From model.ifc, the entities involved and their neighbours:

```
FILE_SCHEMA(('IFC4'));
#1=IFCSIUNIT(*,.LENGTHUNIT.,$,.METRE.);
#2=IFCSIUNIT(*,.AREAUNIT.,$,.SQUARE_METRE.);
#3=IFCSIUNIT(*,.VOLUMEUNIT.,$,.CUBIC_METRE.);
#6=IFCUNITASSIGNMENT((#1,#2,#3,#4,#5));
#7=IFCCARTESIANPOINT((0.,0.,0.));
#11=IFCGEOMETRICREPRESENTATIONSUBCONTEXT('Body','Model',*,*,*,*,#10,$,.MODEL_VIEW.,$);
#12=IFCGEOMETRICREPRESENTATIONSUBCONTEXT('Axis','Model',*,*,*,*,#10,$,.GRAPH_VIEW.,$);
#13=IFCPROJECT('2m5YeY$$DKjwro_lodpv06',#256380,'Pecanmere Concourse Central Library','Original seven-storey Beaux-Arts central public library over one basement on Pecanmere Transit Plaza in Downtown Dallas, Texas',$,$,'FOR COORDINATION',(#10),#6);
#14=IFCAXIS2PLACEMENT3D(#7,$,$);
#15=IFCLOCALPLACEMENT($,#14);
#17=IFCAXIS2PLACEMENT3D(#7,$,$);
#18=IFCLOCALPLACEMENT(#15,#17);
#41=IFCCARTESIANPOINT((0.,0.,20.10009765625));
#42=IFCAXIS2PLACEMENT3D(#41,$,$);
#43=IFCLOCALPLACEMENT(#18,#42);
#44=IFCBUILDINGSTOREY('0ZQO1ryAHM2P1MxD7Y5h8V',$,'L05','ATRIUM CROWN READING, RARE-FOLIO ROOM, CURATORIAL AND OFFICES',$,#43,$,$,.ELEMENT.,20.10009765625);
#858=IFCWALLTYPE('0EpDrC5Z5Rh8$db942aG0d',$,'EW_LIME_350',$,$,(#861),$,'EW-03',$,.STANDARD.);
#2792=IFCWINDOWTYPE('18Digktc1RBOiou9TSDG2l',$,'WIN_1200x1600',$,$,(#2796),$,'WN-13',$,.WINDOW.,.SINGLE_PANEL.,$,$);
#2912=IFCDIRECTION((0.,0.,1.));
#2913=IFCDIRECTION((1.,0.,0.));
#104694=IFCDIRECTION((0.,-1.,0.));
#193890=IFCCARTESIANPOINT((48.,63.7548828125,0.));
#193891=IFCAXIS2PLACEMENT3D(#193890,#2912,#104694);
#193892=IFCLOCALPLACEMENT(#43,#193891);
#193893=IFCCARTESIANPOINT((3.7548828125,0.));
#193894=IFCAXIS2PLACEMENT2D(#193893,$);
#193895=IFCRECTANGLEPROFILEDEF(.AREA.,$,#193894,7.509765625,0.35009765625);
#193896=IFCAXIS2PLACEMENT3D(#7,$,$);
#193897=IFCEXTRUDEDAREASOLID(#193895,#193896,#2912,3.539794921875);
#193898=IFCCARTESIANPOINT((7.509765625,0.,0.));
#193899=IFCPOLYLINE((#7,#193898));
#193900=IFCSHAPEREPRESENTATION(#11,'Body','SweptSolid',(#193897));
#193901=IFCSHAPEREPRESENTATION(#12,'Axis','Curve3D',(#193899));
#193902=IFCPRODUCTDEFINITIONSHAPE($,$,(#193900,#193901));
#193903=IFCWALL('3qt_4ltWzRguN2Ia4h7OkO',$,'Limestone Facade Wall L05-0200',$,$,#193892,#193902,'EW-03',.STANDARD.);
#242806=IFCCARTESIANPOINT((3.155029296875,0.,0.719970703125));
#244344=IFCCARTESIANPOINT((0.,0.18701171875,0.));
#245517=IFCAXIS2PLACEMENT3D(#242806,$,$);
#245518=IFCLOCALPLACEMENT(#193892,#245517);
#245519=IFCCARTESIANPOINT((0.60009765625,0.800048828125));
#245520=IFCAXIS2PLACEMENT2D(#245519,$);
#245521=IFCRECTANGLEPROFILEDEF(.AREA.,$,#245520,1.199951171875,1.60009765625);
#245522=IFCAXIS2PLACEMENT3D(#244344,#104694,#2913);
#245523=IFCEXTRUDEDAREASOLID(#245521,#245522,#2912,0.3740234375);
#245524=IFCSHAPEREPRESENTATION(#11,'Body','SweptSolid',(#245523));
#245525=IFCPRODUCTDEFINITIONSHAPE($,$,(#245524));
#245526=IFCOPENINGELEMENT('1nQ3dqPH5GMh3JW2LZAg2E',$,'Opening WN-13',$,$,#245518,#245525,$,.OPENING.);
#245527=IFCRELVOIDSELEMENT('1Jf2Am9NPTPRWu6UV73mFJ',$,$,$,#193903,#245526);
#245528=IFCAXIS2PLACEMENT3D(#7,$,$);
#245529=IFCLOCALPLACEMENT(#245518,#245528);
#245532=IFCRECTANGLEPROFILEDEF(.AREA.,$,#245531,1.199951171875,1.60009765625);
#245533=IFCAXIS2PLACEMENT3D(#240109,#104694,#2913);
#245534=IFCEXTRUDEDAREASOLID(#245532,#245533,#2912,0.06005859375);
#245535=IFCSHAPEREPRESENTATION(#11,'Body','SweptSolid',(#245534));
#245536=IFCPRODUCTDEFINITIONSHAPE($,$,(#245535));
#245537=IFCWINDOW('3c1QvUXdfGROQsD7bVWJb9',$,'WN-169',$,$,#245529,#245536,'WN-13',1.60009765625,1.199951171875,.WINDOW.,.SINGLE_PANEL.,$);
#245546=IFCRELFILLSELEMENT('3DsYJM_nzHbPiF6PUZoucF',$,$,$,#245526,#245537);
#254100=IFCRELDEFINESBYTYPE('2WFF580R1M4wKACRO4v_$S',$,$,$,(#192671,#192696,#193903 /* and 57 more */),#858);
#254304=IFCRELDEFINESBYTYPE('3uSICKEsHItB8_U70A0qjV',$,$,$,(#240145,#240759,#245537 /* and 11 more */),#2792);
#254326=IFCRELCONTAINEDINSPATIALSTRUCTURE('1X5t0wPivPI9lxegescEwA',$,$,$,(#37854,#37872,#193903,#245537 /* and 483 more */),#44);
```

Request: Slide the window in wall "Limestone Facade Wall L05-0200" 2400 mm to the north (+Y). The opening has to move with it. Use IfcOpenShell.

```python
import ifcopenshell
import ifcopenshell.api.geometry
import ifcopenshell.util.placement
import ifcopenshell.util.unit

model = ifcopenshell.open("model.ifc")
unit_scale = ifcopenshell.util.unit.calculate_unit_scale(model)

window = model.by_id(245537)
opening = window.FillsVoids[0].RelatingOpeningElement
wall = opening.VoidsElements[0].RelatingBuildingElement

wall_matrix = ifcopenshell.util.placement.get_local_placement(wall.ObjectPlacement)
shift = wall_matrix[:3, 0] * -2.4 / unit_scale
before = ifcopenshell.util.placement.get_local_placement(window.ObjectPlacement)[:3, 3].copy()

# The window is placed relative to its opening, so it follows when the opening moves.
matrix = ifcopenshell.util.placement.get_local_placement(opening.ObjectPlacement)
matrix[:3, 3] += shift
ifcopenshell.api.geometry.edit_object_placement(
    model, product=opening, matrix=matrix, is_si=False, should_transform_children=True
)

after = ifcopenshell.util.placement.get_local_placement(window.ObjectPlacement)[:3, 3]
print("window moved by", (after - before).round(3) + 0.0)

model.write("model_rev.ifc")
```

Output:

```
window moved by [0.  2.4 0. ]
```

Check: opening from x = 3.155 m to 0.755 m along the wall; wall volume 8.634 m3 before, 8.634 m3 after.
